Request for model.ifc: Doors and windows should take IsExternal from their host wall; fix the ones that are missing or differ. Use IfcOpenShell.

First a look at what the model holds.

```python
import ifcopenshell
import ifcopenshell.util.element

model = ifcopenshell.open("model.ifc")
print(model.schema)
seen = {}
for e in model.by_type("IfcDoor") + model.by_type("IfcWindow"):
    if not e.FillsVoids:
        continue
    host = e.FillsVoids[0].RelatingOpeningElement.VoidsElements[0].RelatingBuildingElement
    own = ifcopenshell.util.element.get_pset(e, f"Pset_{e.is_a()[3:].removesuffix('StandardCase')}Common", "IsExternal")
    wall = ifcopenshell.util.element.get_pset(host, "Pset_WallCommon", "IsExternal")
    seen[e.is_a(), own, wall] = seen.get((e.is_a(), own, wall), 0) + 1
for (cls, own, wall), count in sorted(seen.items(), key=str):
    print(count, cls, "IsExternal:", own, "| host wall:", wall)
```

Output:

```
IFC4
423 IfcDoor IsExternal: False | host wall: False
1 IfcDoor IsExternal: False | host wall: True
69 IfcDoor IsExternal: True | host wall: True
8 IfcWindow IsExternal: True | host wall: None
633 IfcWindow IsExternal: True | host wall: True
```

```python
import ifcopenshell
import ifcopenshell.api.pset
import ifcopenshell.util.element

model = ifcopenshell.open("model.ifc")

count = 0
for ifc_class, pset_name in (("IfcDoor", "Pset_DoorCommon"), ("IfcWindow", "Pset_WindowCommon")):
    for e in model.by_type(ifc_class):
        if not e.FillsVoids:
            continue
        host = e.FillsVoids[0].RelatingOpeningElement.VoidsElements[0].RelatingBuildingElement
        external = ifcopenshell.util.element.get_pset(host, "Pset_WallCommon", "IsExternal")
        if external is None or ifcopenshell.util.element.get_pset(e, pset_name, "IsExternal") == external:
            continue
        pset = ifcopenshell.api.pset.add_pset(model, product=e, name=pset_name)
        ifcopenshell.api.pset.edit_pset(model, pset=pset, properties={"IsExternal": external})
        count += 1

print(count, "updated")

model.write("model_v2.ifc")
```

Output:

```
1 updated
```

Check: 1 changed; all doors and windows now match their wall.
